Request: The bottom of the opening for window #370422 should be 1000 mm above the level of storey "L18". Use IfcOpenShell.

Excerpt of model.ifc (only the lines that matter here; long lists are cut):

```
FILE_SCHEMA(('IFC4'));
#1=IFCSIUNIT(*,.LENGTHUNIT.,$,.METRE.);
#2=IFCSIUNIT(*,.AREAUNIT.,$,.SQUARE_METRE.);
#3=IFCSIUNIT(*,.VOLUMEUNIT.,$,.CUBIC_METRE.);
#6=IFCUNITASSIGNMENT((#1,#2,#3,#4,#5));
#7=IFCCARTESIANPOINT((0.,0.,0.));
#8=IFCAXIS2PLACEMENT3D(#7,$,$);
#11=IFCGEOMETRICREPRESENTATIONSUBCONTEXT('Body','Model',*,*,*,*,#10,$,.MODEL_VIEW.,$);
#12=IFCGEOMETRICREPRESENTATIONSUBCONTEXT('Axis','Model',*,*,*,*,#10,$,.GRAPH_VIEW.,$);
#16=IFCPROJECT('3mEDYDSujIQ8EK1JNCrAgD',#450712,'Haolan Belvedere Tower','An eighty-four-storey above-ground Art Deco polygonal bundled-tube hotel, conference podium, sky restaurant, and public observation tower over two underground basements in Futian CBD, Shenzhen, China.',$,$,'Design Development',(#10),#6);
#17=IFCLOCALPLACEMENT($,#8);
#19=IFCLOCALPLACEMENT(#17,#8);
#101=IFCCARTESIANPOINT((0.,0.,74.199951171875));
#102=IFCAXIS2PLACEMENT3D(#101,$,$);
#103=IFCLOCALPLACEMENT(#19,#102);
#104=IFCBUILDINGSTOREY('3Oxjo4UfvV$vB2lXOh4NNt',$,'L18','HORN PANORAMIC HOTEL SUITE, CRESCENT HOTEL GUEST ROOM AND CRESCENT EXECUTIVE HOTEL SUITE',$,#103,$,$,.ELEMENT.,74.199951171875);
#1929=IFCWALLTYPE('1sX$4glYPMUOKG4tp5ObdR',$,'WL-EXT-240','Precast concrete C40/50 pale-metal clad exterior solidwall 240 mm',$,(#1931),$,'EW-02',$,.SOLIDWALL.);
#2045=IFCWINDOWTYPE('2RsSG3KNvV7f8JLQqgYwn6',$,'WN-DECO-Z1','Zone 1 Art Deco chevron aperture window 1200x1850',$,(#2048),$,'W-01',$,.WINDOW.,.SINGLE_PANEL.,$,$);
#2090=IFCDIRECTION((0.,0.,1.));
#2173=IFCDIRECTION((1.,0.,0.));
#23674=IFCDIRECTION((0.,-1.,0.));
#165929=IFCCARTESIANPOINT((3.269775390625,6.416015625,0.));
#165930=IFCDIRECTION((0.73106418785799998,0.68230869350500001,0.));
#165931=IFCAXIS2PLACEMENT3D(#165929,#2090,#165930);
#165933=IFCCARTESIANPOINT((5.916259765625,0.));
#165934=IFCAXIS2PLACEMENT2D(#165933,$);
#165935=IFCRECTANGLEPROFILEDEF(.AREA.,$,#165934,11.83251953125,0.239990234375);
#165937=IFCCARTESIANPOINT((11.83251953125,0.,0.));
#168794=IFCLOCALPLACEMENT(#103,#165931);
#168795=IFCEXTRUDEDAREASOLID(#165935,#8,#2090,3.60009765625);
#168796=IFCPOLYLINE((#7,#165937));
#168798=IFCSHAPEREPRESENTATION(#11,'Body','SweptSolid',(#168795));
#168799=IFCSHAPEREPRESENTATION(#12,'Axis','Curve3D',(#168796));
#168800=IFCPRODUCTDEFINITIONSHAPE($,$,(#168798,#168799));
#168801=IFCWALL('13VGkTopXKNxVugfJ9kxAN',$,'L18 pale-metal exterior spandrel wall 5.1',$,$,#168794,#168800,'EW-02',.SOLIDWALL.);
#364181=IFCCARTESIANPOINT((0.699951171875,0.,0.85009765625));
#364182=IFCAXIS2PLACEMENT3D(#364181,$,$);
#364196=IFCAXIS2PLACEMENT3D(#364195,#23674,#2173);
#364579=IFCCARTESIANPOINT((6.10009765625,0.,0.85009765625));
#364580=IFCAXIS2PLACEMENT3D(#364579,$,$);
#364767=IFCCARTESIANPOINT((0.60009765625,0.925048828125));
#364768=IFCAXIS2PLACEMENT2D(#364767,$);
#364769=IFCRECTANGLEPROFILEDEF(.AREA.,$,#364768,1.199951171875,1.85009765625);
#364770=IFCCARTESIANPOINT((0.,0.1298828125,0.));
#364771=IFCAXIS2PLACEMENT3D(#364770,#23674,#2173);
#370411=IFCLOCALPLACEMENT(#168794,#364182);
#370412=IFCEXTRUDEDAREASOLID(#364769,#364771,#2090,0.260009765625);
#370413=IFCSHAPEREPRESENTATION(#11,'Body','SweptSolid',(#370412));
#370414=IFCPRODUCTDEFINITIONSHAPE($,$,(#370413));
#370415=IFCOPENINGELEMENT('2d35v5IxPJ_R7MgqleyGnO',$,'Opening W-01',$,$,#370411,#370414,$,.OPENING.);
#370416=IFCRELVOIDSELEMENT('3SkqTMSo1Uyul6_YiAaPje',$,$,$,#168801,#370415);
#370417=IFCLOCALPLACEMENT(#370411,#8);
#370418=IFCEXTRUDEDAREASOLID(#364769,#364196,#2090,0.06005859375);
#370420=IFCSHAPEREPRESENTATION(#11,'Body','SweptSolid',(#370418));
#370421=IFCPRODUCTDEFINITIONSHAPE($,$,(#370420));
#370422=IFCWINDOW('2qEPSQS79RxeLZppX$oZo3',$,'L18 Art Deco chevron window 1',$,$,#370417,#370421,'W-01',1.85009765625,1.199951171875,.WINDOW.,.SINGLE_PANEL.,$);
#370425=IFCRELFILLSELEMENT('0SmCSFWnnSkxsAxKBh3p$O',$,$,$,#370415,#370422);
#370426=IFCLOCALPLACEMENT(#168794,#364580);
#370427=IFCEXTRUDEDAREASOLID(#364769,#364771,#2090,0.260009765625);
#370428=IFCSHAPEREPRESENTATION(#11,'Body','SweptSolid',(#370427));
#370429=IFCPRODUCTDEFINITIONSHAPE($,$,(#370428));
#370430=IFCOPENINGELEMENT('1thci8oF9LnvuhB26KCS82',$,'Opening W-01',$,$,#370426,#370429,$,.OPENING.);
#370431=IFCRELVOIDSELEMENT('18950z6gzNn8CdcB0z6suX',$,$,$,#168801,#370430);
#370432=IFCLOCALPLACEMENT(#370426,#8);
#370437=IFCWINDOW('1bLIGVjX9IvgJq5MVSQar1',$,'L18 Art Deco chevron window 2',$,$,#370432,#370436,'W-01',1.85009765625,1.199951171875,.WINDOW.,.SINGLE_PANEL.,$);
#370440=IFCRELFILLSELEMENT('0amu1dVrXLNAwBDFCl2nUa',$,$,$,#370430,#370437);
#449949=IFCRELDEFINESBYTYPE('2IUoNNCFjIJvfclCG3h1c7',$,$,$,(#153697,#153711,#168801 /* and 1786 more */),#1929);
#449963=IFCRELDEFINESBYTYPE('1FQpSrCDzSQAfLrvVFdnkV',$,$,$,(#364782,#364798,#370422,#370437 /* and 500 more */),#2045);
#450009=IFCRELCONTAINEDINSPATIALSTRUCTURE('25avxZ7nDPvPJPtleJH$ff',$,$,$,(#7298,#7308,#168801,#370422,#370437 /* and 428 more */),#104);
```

```python
import numpy as np
import ifcopenshell
import ifcopenshell.api.geometry
import ifcopenshell.geom
import ifcopenshell.util.element
import ifcopenshell.util.placement
import ifcopenshell.util.shape
import ifcopenshell.util.unit

model = ifcopenshell.open("model.ifc")
unit_scale = ifcopenshell.util.unit.calculate_unit_scale(model)

window = model.by_id(370422)
opening = window.FillsVoids[0].RelatingOpeningElement
storey = ifcopenshell.util.element.get_container(window, ifc_class="IfcBuildingStorey")
level = ifcopenshell.util.placement.get_local_placement(storey.ObjectPlacement)[2, 3]

# The opening's origin need not be at the sill, so measure its lowest point.
shape = ifcopenshell.geom.create_shape(ifcopenshell.geom.settings(), opening)
bottom = ifcopenshell.util.shape.get_shape_bottom_elevation(shape, shape.geometry) / unit_scale
dz = level + 1.0 - bottom

shift = np.array([0.0, 0.0, dz])
# The window is placed relative to its opening, so it follows when the opening moves.
matrix = ifcopenshell.util.placement.get_local_placement(opening.ObjectPlacement)
matrix[:3, 3] += shift
ifcopenshell.api.geometry.edit_object_placement(
    model, product=opening, matrix=matrix, is_si=False, should_transform_children=True
)

print(f"moved by {dz * unit_scale:+.3f} m")

model.write("model_rev.ifc")
```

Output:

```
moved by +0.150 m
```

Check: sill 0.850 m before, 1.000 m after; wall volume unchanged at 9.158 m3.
